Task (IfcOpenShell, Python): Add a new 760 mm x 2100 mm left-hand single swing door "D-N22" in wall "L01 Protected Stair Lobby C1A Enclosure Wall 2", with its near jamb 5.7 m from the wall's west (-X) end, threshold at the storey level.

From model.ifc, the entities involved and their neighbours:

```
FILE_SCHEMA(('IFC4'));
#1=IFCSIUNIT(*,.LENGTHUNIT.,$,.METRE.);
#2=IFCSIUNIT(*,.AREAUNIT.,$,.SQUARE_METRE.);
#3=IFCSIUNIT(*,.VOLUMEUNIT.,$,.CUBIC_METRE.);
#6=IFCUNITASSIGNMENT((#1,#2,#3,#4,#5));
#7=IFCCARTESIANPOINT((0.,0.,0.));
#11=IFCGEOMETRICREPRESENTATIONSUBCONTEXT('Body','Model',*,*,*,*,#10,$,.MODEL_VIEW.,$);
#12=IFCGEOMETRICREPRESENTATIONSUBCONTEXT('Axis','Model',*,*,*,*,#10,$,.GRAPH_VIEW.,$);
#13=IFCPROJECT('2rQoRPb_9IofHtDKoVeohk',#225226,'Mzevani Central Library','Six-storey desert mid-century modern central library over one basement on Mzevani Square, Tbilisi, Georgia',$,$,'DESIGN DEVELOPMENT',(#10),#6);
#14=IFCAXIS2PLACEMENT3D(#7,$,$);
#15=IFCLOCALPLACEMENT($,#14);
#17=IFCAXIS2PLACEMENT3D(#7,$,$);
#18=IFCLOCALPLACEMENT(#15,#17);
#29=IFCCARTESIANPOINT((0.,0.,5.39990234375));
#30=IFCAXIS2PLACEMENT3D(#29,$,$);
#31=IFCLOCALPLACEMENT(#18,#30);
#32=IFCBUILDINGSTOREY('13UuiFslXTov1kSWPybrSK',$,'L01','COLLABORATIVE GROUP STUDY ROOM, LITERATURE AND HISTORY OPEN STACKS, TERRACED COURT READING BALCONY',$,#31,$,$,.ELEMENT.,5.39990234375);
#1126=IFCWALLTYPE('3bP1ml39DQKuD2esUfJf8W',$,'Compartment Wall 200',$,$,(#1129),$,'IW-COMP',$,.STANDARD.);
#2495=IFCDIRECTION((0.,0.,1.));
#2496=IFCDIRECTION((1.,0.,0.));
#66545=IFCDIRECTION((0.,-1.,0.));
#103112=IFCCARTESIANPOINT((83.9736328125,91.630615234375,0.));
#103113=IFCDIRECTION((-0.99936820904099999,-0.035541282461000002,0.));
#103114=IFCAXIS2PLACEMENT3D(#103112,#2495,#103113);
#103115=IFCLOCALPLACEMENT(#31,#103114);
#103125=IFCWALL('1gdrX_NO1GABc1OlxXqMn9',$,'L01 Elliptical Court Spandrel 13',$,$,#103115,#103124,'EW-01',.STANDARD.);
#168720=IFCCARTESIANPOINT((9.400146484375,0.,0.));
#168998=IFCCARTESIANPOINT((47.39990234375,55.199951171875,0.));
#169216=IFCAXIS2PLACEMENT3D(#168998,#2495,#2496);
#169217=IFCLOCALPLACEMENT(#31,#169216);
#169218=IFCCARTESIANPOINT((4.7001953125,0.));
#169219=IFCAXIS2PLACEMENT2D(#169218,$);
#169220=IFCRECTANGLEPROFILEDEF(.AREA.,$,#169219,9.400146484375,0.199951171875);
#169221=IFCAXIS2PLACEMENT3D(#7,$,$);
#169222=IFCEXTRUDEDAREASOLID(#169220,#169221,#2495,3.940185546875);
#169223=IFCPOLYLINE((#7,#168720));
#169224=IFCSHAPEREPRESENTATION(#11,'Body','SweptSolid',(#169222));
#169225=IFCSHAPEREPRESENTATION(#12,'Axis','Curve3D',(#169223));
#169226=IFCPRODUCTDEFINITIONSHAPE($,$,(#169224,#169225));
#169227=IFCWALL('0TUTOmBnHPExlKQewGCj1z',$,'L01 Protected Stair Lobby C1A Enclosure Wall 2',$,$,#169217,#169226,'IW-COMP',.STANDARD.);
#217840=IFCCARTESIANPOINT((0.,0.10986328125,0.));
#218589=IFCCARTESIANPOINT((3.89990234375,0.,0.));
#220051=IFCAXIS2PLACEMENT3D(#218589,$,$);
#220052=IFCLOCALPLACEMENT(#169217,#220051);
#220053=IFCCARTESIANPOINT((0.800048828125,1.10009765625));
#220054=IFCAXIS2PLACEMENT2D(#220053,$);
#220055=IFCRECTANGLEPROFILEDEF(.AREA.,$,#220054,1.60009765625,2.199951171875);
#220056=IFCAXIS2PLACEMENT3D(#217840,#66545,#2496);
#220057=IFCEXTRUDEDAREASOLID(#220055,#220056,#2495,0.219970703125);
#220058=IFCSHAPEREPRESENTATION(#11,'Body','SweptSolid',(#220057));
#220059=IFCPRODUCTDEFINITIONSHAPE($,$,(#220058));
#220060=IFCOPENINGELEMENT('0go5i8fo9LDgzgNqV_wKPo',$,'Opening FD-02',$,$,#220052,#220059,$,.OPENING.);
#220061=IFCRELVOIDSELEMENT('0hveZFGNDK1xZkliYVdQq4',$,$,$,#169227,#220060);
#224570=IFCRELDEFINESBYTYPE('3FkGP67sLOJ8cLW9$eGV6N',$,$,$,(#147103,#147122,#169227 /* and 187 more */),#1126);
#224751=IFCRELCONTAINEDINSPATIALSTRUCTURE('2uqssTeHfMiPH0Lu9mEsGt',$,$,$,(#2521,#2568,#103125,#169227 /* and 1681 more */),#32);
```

```python
import numpy as np
import ifcopenshell
import ifcopenshell.api.feature
import ifcopenshell.api.geometry
import ifcopenshell.api.root
import ifcopenshell.api.spatial
import ifcopenshell.geom
import ifcopenshell.util.element
import ifcopenshell.util.placement
import ifcopenshell.util.representation
import ifcopenshell.util.shape
import ifcopenshell.util.unit

model = ifcopenshell.open("model.ifc")
unit_scale = ifcopenshell.util.unit.calculate_unit_scale(model)
settings = ifcopenshell.geom.settings()


def volume(element):
    """Net volume in cubic metres, openings subtracted."""
    shape = ifcopenshell.geom.create_shape(settings, element)
    return ifcopenshell.util.shape.get_volume(shape.geometry)


wall = model.by_id(169227)
storey = ifcopenshell.util.element.get_container(wall, ifc_class="IfcBuildingStorey")
context = ifcopenshell.util.representation.get_context(model, "Model", "Body", "MODEL_VIEW")
before = volume(wall)

width, height, from_end, sill = 0.76, 2.1, 5.7, 0.0  # metres

# The wall runs along its own X axis, and the end named is its -X end.
wall_shape = ifcopenshell.geom.create_shape(settings, wall)
x, y, z = ifcopenshell.util.shape.get_vertices(wall_shape.geometry).T
start = x.min() + from_end
face, thickness = float(y.min()), float(y.max() - y.min())
wall_matrix = ifcopenshell.util.placement.get_local_placement(wall.ObjectPlacement)
level = ifcopenshell.util.placement.get_local_placement(storey.ObjectPlacement)[2, 3]


def in_wall(x, y):
    """Placement at x, y metres in the wall's axes, at sill height."""
    matrix = wall_matrix.copy()
    matrix[:, 3] = wall_matrix @ np.array([x / unit_scale, y / unit_scale, 0.0, 1.0])
    matrix[2, 3] = level + sill / unit_scale
    return matrix


# Opening: a box that overshoots both wall faces by 50 mm.
opening = ifcopenshell.api.root.create_entity(model, ifc_class="IfcOpeningElement", predefined_type="OPENING")
box = ifcopenshell.api.geometry.add_wall_representation(
    model, context=context, length=width, height=height, thickness=thickness + 0.1
)
ifcopenshell.api.geometry.assign_representation(model, product=opening, representation=box)
ifcopenshell.api.geometry.edit_object_placement(model, product=opening, matrix=in_wall(start, face - 0.05), is_si=False)
ifcopenshell.api.feature.add_feature(model, feature=opening, element=wall)

door = ifcopenshell.api.root.create_entity(model, ifc_class="IfcDoor", name="D-N22", predefined_type="DOOR")
door.OverallWidth, door.OverallHeight = width / unit_scale, height / unit_scale
door.OperationType = "SINGLE_SWING_LEFT"
body = ifcopenshell.api.geometry.add_door_representation(
    model,
    context=context,
    overall_width=door.OverallWidth,
    overall_height=door.OverallHeight,
    operation_type="SINGLE_SWING_LEFT",
    lining_properties={"LiningDepth": thickness / unit_scale, "ThresholdDepth": thickness / unit_scale},
)
ifcopenshell.api.geometry.assign_representation(model, product=door, representation=body)
ifcopenshell.api.spatial.assign_container(model, products=[door], relating_structure=storey)
ifcopenshell.api.feature.add_filling(model, opening=opening, element=door)

# The lining spans the wall, so the door starts at the wall face.
ifcopenshell.api.geometry.edit_object_placement(model, product=door, matrix=in_wall(start, face), is_si=False)

after = volume(wall)

print(f"wall volume {before:.3f} -> {after:.3f} m3")

model.write("model_edited.ifc")
```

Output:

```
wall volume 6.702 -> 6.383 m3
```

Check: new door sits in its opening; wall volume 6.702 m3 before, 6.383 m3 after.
